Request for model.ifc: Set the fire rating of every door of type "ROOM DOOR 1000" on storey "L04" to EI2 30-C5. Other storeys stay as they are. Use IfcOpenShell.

First a look at what the model holds.

```python
import ifcopenshell
import ifcopenshell.util.element

model = ifcopenshell.open("model.ifc")
print(model.schema)
storey = next(s for s in model.by_type("IfcBuildingStorey") if s.Name == "L04")
doors = [e for e in ifcopenshell.util.element.get_decomposition(storey) if e.is_a("IfcDoor")]
seen = {}
for e in doors:
    element_type = ifcopenshell.util.element.get_type(e)
    key = (element_type.Name if element_type != e and element_type else None, ifcopenshell.util.element.get_pset(e, "Pset_DoorCommon", "FireRating"))
    seen[key] = seen.get(key, 0) + 1
for (name, value), count in sorted(seen.items(), key=str):
    print(count, "x", name, "|", value)
```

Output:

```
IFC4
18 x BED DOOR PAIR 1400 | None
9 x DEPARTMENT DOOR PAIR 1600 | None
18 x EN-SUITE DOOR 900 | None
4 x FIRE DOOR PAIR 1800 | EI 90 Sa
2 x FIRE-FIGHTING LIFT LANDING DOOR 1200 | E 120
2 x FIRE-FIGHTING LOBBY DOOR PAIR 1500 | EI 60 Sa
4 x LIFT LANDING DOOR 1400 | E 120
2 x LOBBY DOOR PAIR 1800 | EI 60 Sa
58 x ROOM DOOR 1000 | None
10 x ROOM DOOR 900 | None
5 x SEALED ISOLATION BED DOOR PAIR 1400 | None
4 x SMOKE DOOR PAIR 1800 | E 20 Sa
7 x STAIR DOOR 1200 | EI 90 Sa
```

```python
import ifcopenshell
import ifcopenshell.api.pset
import ifcopenshell.util.element

model = ifcopenshell.open("model.ifc")

storey = next(s for s in model.by_type("IfcBuildingStorey") if s.Name == "L04")
doors = [e for e in ifcopenshell.util.element.get_decomposition(storey) if e.is_a("IfcDoor")]

count = 0
for e in doors:
    element_type = ifcopenshell.util.element.get_type(e)
    if element_type in (None, e) or element_type.Name != "ROOM DOOR 1000":
        continue
    # add_pset returns the element's existing set when there is one.
    pset = ifcopenshell.api.pset.add_pset(model, product=e, name="Pset_DoorCommon")
    ifcopenshell.api.pset.edit_pset(model, pset=pset, properties={"FireRating": "EI2 30-C5"})
    count += 1

print(count, "doors updated")

model.write("model_rev.ifc")
```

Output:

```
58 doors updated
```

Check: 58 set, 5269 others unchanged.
